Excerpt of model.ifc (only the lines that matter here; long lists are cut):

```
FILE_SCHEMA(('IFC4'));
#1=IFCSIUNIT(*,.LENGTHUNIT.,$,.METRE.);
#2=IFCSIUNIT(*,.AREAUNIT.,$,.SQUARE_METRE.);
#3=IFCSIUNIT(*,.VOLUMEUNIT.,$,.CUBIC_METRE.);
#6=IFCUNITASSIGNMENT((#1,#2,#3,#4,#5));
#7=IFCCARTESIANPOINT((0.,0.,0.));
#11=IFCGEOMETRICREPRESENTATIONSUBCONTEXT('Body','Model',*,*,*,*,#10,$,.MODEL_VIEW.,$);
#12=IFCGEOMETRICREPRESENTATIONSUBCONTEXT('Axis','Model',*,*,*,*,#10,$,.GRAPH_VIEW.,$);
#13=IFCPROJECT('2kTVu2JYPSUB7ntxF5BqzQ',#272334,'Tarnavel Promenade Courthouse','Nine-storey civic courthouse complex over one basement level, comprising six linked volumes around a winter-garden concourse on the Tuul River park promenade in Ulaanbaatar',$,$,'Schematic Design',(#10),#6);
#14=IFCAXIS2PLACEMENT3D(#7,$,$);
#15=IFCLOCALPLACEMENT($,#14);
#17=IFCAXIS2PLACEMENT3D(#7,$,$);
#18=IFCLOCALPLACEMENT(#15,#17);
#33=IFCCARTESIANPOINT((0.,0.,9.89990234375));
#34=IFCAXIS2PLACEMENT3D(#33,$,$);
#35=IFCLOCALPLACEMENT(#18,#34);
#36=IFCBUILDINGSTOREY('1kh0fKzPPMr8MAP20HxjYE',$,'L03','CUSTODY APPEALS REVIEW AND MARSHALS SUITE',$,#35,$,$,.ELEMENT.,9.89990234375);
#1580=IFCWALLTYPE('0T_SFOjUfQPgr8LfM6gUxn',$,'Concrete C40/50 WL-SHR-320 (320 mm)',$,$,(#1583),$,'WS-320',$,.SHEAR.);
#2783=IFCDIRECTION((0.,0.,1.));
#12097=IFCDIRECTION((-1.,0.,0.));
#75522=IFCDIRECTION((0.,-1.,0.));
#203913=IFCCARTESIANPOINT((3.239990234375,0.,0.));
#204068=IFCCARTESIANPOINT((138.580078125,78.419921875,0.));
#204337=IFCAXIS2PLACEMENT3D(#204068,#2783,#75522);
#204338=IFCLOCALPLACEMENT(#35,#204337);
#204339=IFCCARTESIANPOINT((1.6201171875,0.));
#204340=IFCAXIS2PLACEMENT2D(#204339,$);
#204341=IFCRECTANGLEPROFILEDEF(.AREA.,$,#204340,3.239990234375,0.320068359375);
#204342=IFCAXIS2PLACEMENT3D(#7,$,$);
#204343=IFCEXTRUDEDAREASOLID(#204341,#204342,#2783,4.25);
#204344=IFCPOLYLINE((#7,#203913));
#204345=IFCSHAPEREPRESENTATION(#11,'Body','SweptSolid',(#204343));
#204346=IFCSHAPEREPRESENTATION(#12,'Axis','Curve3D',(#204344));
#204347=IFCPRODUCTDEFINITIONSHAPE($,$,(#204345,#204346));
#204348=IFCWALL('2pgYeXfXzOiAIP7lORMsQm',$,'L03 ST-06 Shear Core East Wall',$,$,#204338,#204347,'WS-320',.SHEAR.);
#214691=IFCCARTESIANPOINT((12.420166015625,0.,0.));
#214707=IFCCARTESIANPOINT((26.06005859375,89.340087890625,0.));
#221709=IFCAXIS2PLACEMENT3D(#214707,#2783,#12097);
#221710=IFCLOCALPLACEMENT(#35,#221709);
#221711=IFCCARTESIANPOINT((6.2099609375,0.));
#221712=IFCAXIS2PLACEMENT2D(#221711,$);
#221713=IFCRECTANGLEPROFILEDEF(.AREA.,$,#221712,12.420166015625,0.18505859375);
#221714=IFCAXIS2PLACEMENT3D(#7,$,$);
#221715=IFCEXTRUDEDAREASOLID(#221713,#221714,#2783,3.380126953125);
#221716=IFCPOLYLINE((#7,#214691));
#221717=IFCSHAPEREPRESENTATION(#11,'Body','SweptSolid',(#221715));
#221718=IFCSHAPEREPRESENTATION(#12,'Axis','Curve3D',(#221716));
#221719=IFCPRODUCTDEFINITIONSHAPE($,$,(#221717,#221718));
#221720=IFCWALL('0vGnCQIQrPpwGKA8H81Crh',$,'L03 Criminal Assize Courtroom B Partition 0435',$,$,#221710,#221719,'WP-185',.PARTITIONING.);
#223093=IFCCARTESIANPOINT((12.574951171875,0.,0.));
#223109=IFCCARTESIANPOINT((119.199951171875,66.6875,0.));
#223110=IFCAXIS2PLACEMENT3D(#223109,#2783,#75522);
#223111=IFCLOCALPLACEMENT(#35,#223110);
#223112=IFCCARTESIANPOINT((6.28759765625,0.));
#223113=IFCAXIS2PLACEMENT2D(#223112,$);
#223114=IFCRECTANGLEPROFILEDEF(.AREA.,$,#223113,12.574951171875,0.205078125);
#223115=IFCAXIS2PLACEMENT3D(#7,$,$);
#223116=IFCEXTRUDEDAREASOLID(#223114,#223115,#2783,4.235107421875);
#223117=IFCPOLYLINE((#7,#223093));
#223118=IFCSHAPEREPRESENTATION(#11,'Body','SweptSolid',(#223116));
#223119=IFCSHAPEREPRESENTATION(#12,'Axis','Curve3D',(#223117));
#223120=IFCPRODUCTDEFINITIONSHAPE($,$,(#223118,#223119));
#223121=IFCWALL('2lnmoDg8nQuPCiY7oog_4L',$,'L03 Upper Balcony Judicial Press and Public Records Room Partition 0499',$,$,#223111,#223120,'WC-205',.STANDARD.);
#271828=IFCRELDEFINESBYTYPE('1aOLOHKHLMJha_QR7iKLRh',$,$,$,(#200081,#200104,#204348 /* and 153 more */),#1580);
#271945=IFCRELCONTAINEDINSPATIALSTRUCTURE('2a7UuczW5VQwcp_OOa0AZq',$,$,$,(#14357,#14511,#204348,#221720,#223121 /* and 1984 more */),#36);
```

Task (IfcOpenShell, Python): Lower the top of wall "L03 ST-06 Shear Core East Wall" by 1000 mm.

```python
import ifcopenshell
import ifcopenshell.geom
import ifcopenshell.util.representation
import ifcopenshell.util.shape

model = ifcopenshell.open("model.ifc")
settings = ifcopenshell.geom.settings()


def volume(element):
    """Net volume in cubic metres, openings subtracted."""
    shape = ifcopenshell.geom.create_shape(settings, element)
    return ifcopenshell.util.shape.get_volume(shape.geometry)


wall = model.by_id(204348)
before = volume(wall)

body = ifcopenshell.util.representation.get_representation(wall, "Model", "Body")
solid = body.Items[0]
old_height = solid.Depth
solid.Depth -= 1.0
after = volume(wall)

print(f"height {old_height:g} -> {solid.Depth:g}, volume {before:.3f} -> {after:.3f} m3")

model.write("model_rev.ifc")
```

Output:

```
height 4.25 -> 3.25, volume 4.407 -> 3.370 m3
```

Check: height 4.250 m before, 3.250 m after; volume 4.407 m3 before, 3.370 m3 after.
